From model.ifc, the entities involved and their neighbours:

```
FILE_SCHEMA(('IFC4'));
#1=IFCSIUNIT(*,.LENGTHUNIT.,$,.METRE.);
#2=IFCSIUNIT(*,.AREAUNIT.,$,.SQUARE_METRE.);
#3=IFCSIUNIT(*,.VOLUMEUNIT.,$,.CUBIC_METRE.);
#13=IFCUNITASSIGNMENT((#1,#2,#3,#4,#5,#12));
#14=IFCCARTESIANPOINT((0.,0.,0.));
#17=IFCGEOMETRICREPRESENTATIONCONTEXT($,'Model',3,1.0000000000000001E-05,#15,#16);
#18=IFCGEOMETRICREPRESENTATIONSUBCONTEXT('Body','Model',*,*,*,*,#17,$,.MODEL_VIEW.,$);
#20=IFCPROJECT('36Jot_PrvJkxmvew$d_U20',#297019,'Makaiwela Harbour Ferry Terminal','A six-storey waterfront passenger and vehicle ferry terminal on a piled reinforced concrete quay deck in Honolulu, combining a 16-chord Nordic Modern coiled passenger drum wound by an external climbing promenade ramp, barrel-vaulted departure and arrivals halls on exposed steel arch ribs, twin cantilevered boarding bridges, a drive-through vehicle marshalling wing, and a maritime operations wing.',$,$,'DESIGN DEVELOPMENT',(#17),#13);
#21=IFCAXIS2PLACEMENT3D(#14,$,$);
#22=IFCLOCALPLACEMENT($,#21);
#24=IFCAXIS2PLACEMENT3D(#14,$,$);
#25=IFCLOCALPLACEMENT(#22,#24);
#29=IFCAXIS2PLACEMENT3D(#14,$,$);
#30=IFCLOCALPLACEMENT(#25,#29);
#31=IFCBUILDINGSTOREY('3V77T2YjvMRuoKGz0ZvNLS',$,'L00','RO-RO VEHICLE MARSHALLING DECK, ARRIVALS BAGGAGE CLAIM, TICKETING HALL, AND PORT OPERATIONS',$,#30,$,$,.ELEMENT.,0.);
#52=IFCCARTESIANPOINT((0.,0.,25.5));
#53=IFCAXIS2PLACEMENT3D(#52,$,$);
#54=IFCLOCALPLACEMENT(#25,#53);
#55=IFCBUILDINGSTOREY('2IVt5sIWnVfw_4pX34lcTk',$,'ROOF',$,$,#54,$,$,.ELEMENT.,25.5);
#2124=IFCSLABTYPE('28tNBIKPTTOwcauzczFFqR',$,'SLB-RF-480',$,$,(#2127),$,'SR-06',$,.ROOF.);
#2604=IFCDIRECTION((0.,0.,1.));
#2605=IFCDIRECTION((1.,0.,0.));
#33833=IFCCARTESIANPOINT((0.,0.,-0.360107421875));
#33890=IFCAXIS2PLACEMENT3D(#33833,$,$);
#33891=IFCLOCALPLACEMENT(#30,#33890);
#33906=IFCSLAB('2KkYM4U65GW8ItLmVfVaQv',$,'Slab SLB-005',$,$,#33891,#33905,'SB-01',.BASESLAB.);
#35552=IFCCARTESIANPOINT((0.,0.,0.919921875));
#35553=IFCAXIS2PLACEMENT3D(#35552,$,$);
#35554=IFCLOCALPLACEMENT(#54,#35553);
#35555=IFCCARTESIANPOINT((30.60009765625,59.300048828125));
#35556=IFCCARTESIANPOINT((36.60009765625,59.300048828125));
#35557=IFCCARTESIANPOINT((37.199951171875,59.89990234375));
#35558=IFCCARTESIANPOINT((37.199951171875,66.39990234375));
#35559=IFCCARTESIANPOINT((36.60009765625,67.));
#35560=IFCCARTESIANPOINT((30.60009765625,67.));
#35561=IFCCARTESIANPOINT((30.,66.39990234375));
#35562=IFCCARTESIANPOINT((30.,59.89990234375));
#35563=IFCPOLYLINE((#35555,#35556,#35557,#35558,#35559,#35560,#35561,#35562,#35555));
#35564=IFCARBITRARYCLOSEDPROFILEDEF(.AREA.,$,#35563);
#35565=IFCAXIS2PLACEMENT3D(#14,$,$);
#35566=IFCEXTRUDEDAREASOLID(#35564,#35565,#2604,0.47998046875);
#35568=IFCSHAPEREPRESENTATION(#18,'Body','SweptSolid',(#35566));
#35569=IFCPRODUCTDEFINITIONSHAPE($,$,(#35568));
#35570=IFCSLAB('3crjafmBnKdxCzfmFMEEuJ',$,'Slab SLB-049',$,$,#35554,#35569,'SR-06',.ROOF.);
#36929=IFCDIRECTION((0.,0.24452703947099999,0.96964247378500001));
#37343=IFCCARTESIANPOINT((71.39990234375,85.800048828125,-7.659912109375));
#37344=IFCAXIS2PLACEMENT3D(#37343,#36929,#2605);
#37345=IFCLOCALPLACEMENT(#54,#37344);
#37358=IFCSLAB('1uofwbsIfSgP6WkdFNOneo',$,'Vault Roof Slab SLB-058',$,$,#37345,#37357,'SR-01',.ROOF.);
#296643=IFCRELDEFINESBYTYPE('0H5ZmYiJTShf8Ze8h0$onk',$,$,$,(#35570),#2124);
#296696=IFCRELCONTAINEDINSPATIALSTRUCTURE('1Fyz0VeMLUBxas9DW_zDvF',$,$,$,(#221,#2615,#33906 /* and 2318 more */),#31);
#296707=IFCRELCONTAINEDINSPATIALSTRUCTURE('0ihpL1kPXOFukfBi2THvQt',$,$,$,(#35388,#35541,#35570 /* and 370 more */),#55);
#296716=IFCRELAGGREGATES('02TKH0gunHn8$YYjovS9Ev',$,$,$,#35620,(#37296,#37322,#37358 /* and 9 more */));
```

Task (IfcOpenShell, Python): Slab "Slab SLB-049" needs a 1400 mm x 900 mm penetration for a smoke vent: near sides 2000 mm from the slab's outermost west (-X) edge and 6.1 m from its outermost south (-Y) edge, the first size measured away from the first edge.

```python
import numpy as np
import ifcopenshell
import ifcopenshell.api.feature
import ifcopenshell.api.geometry
import ifcopenshell.api.root
import ifcopenshell.geom
import ifcopenshell.util.placement
import ifcopenshell.util.representation
import ifcopenshell.util.shape
import ifcopenshell.util.unit

model = ifcopenshell.open("model.ifc")
unit_scale = ifcopenshell.util.unit.calculate_unit_scale(model)
settings = ifcopenshell.geom.settings()


def volume(element):
    """Net volume in cubic metres, openings subtracted."""
    shape = ifcopenshell.geom.create_shape(settings, element)
    return ifcopenshell.util.shape.get_volume(shape.geometry)


slab = model.by_guid("3crjafmBnKdxCzfmFMEEuJ")
before = volume(slab)

# Extent in the slab's own axes, in metres. The edges named are its -X and -Y sides.
slab_shape = ifcopenshell.geom.create_shape(settings, slab)
vertices = ifcopenshell.util.shape.get_vertices(slab_shape.geometry)
x_min, y_min, bottom = vertices.min(axis=0)
top = vertices[:, 2].max()

opening = ifcopenshell.api.root.create_entity(model, ifc_class="IfcOpeningElement", name="Smoke vent opening", predefined_type="OPENING")
context = ifcopenshell.util.representation.get_context(model, "Model", "Body", "MODEL_VIEW")
width, depth = 1.4, 0.9
outline = [(0.0, 0.0), (width, 0.0), (width, depth), (0.0, depth), (0.0, 0.0)]
# Overshoot both faces by 50 mm so the cut is clean.
shape = ifcopenshell.api.geometry.add_slab_representation(
    model, context=context, depth=top - bottom + 0.1, polyline=outline
)
ifcopenshell.api.geometry.assign_representation(model, product=opening, representation=shape)

matrix = ifcopenshell.util.placement.get_local_placement(slab.ObjectPlacement)
matrix[:, 3] = matrix @ np.append(np.array([x_min + 2, y_min + 6.1, bottom - 0.05]) / unit_scale, 1.0)
ifcopenshell.api.geometry.edit_object_placement(model, product=opening, matrix=matrix, is_si=False)
ifcopenshell.api.feature.add_feature(model, feature=opening, element=slab)

after = volume(slab)

print(f"slab volume {before:.3f} -> {after:.3f} m3")

model.write("model_edited.ifc")
```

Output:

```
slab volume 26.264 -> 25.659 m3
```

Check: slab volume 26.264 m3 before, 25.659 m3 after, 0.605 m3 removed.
